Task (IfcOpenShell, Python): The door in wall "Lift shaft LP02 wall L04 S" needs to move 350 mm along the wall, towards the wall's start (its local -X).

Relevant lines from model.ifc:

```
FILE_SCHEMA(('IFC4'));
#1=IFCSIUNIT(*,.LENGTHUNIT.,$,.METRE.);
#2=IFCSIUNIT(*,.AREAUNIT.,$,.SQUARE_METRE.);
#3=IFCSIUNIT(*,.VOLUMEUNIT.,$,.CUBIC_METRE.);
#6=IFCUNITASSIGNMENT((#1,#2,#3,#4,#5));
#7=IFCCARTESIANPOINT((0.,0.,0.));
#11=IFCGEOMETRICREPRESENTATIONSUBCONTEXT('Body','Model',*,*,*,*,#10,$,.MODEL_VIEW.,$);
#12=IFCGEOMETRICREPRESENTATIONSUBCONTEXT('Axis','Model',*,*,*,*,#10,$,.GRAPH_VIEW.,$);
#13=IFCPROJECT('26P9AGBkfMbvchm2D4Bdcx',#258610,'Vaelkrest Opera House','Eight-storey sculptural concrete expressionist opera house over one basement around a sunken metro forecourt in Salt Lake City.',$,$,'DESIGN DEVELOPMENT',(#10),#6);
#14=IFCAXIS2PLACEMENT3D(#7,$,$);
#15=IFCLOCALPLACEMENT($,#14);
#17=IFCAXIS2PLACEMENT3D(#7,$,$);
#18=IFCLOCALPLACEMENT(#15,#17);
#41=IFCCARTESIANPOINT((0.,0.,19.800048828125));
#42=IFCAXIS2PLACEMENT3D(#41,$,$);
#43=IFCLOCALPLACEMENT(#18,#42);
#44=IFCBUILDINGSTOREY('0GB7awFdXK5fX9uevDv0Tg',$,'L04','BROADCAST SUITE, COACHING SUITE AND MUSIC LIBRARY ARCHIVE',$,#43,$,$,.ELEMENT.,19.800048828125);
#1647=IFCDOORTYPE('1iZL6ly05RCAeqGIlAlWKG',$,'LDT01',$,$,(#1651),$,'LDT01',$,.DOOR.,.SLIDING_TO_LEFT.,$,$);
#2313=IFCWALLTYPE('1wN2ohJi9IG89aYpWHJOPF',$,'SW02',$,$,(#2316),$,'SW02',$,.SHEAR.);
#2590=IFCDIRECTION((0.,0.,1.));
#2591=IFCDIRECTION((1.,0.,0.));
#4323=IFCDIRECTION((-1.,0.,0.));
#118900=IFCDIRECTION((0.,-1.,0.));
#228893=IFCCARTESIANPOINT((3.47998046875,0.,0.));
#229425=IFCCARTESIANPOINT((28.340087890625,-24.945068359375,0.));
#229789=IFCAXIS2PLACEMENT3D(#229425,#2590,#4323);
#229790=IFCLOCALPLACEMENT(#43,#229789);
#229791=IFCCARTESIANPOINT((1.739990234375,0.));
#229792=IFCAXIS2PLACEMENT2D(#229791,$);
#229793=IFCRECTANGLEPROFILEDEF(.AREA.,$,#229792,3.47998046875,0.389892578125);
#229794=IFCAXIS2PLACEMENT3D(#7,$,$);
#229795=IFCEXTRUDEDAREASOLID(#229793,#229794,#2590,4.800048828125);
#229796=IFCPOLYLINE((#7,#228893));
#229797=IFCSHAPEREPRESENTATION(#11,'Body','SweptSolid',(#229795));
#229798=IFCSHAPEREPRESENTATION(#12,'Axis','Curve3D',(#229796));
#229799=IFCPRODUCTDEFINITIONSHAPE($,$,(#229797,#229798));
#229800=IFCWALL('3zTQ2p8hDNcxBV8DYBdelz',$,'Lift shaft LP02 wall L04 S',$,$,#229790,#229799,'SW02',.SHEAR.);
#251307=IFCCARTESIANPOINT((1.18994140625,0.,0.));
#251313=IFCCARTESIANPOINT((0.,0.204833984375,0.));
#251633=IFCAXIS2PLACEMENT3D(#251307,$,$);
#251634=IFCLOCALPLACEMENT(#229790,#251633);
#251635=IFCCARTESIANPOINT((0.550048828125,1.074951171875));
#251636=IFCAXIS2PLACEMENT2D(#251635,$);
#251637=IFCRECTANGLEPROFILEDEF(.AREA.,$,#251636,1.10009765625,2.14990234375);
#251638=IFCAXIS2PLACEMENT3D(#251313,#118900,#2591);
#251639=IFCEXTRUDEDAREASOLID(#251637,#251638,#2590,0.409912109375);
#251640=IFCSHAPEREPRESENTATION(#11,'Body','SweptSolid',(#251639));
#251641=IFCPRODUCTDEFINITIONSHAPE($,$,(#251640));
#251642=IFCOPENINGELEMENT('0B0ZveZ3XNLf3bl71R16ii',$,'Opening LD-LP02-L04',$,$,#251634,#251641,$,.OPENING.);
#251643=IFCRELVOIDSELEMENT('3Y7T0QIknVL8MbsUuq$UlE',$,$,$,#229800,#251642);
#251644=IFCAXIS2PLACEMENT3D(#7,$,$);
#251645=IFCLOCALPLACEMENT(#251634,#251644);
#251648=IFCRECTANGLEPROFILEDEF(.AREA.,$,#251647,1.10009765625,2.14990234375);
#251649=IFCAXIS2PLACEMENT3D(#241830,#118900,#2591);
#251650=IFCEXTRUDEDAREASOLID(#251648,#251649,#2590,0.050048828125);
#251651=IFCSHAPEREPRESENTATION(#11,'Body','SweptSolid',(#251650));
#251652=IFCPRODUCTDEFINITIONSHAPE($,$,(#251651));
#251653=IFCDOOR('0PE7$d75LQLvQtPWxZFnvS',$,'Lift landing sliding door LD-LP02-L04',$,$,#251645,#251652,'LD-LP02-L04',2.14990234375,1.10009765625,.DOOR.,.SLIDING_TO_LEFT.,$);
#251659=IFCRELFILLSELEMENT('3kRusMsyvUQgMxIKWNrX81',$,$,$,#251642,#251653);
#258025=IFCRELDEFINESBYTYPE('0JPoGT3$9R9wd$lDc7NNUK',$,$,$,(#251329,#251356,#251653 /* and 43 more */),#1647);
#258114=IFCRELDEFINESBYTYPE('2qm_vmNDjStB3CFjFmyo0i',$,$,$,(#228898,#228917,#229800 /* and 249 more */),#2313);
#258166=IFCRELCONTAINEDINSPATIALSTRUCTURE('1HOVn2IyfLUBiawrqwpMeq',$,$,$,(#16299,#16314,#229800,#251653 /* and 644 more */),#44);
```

```python
import ifcopenshell
import ifcopenshell.api.geometry
import ifcopenshell.util.placement

model = ifcopenshell.open("model.ifc")

door = model.by_guid("0PE7$d75LQLvQtPWxZFnvS")
opening = door.FillsVoids[0].RelatingOpeningElement
wall = opening.VoidsElements[0].RelatingBuildingElement

wall_matrix = ifcopenshell.util.placement.get_local_placement(wall.ObjectPlacement)
shift = wall_matrix[:3, 0] * -0.35
before = ifcopenshell.util.placement.get_local_placement(door.ObjectPlacement)[:3, 3].copy()

# The door is placed relative to its opening, so it follows when the opening moves.
matrix = ifcopenshell.util.placement.get_local_placement(opening.ObjectPlacement)
matrix[:3, 3] += shift
ifcopenshell.api.geometry.edit_object_placement(
    model, product=opening, matrix=matrix, is_si=False, should_transform_children=True
)

after = ifcopenshell.util.placement.get_local_placement(door.ObjectPlacement)[:3, 3]
print("door moved by", (after - before).round(3) + 0.0)

model.write("model_edited.ifc")
```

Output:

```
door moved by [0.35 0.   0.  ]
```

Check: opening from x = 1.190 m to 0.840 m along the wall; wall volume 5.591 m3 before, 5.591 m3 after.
